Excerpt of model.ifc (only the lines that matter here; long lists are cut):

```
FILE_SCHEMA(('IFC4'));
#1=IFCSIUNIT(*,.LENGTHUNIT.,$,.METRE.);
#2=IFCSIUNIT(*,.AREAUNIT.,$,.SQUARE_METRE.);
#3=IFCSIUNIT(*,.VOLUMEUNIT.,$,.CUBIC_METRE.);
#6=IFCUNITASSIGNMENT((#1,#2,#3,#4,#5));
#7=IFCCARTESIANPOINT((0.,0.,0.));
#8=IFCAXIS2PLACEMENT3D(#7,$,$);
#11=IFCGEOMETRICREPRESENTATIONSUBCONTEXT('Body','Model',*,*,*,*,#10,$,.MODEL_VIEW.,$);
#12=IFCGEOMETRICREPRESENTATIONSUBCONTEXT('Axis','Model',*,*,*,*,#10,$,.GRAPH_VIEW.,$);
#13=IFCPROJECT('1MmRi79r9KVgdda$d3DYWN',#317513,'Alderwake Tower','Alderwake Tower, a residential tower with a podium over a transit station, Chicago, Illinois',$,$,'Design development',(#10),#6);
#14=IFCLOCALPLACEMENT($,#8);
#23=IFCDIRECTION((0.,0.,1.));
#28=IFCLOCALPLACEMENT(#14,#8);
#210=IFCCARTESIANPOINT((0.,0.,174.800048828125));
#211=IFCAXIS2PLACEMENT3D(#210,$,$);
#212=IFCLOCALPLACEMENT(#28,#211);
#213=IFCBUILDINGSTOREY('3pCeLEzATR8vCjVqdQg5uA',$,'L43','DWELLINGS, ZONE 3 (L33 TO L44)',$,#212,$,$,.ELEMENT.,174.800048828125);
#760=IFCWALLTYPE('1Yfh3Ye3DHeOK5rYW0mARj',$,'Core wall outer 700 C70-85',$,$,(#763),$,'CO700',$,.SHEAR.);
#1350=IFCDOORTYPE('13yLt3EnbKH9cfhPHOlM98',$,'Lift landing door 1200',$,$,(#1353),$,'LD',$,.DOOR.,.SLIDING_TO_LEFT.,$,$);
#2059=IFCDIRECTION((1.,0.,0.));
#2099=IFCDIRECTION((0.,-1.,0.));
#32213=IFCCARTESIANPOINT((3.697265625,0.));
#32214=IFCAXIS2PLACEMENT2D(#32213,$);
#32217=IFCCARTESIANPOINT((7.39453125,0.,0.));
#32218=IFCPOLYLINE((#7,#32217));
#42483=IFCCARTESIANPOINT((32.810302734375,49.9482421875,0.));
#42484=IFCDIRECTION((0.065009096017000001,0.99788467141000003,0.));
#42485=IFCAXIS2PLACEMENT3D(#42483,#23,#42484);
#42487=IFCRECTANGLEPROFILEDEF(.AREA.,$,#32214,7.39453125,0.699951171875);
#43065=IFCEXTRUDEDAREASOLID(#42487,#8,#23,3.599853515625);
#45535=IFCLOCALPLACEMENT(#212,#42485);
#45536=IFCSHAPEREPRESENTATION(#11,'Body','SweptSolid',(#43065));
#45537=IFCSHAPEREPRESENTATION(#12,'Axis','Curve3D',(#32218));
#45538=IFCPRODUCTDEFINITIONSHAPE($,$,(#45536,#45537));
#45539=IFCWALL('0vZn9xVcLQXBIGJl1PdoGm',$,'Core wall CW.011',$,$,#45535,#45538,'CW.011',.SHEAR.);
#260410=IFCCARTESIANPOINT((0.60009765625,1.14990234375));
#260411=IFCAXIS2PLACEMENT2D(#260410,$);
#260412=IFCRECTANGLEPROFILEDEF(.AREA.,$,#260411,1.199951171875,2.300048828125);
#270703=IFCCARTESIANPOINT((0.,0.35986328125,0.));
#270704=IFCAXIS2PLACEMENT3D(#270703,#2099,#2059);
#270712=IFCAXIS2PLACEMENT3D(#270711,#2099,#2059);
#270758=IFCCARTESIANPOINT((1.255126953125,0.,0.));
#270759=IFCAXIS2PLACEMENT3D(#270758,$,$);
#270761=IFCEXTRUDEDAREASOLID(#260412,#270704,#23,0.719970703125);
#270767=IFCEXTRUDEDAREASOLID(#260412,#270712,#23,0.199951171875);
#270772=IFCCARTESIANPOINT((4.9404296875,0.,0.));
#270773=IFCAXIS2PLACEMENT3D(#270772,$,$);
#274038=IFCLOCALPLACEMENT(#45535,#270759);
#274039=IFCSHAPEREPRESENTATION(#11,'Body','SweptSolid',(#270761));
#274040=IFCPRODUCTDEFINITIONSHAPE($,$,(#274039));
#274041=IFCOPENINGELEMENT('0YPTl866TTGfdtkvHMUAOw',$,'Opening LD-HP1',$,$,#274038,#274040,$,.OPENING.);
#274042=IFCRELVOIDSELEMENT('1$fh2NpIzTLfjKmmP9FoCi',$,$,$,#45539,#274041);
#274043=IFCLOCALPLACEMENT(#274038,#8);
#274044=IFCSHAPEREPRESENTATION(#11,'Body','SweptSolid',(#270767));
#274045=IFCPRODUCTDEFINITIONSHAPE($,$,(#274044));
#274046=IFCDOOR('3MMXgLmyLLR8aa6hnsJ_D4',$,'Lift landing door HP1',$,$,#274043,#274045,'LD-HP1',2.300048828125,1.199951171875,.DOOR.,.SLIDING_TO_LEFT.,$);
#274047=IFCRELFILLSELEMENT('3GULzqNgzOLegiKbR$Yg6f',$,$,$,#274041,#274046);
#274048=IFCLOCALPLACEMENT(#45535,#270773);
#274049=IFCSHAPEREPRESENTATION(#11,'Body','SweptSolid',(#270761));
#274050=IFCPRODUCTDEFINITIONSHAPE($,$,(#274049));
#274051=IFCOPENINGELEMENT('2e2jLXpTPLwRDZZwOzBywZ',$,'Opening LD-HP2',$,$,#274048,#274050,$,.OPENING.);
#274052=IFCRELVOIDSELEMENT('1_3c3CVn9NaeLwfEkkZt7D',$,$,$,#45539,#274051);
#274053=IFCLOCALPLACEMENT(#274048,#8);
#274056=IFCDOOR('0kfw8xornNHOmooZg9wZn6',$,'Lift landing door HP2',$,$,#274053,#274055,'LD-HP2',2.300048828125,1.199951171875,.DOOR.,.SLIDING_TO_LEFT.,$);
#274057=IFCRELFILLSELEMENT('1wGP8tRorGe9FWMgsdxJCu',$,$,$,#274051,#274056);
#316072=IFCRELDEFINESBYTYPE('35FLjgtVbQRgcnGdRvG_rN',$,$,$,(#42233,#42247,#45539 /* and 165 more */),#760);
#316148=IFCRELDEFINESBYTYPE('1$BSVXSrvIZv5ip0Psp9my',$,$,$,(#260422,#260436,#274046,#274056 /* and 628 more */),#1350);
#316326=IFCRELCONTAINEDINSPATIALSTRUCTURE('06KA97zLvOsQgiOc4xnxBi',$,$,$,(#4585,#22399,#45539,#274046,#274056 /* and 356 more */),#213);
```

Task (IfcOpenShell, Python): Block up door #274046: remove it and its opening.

```python
import ifcopenshell
import ifcopenshell.api.feature
import ifcopenshell.api.root
import ifcopenshell.geom
import ifcopenshell.util.shape

model = ifcopenshell.open("model.ifc")
settings = ifcopenshell.geom.settings()


def volume(element):
    """Net volume in cubic metres, openings subtracted."""
    shape = ifcopenshell.geom.create_shape(settings, element)
    return ifcopenshell.util.shape.get_volume(shape.geometry)


door = model.by_id(274046)
opening = door.FillsVoids[0].RelatingOpeningElement
wall = opening.VoidsElements[0].RelatingBuildingElement
before = volume(wall)

ifcopenshell.api.root.remove_product(model, product=door)
ifcopenshell.api.feature.remove_feature(model, feature=opening)

after = volume(wall)

print(f"wall volume {before:.3f} -> {after:.3f} m3")

model.write("model_rev.ifc")
```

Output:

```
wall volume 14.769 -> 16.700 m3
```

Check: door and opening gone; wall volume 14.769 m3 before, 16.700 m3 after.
